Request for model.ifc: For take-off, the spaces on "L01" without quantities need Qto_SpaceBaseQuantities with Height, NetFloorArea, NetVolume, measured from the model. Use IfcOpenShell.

First a look at what the model holds.

```python
import ifcopenshell
import ifcopenshell.util.element
import ifcopenshell.util.unit

model = ifcopenshell.open("model.ifc")
print(model.schema)
for unit_type in ("LENGTHUNIT", "AREAUNIT", "VOLUMEUNIT"):
    print(unit_type, ifcopenshell.util.unit.calculate_unit_scale(model, unit_type))
storey = next(s for s in model.by_type("IfcBuildingStorey") if s.Name == "L01")
spaces = [e for e in ifcopenshell.util.element.get_decomposition(storey) if e.is_a("IfcSpace")]
for e in sorted(spaces, key=lambda e: e.id()):
    print(e.id(), e.is_a(), e.Name, list(ifcopenshell.util.element.get_psets(e, qtos_only=True)), sep=" | ")
```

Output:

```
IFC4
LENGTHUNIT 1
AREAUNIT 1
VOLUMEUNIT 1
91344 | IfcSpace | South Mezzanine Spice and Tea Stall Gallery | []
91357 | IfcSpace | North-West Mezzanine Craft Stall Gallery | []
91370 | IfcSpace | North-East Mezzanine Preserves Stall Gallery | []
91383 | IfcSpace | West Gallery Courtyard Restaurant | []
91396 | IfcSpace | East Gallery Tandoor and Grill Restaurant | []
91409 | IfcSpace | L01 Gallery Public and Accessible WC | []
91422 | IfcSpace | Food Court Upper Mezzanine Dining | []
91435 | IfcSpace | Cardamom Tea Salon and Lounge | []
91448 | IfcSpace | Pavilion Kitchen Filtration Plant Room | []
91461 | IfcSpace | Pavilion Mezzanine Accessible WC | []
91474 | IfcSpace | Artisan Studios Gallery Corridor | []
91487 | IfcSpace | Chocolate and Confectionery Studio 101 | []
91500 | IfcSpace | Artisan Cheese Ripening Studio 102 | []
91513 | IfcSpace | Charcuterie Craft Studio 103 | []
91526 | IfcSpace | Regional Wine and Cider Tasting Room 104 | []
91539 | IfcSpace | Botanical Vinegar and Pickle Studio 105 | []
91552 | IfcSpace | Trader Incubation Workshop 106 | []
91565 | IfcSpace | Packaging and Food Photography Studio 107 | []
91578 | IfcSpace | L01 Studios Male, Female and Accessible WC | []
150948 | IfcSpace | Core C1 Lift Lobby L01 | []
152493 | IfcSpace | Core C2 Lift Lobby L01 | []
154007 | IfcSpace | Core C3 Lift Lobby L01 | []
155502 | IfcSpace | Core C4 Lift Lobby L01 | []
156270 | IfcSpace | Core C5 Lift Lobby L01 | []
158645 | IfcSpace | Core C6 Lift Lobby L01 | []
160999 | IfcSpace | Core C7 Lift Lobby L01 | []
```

```python
import ifcopenshell
import ifcopenshell.api.pset
import ifcopenshell.geom
import ifcopenshell.util.element
import ifcopenshell.util.shape
import ifcopenshell.util.unit

model = ifcopenshell.open("model.ifc")
unit_scale = ifcopenshell.util.unit.calculate_unit_scale(model)
area_scale = ifcopenshell.util.unit.calculate_unit_scale(model, "AREAUNIT")
volume_scale = ifcopenshell.util.unit.calculate_unit_scale(model, "VOLUMEUNIT")
settings = ifcopenshell.geom.settings()

storey = next(s for s in model.by_type("IfcBuildingStorey") if s.Name == "L01")
spaces = [e for e in ifcopenshell.util.element.get_decomposition(storey) if e.is_a("IfcSpace")]

for e in sorted(spaces, key=lambda e: e.id()):
    if ifcopenshell.util.element.get_psets(e, qtos_only=True, should_inherit=False):
        continue
    # Geometry comes back in metres, in the element's own axes.
    shape = ifcopenshell.geom.create_shape(settings, e)
    values = {
        "Height": ifcopenshell.util.shape.get_z(shape.geometry) / unit_scale,
        "NetFloorArea": ifcopenshell.util.shape.get_footprint_area(shape.geometry) / area_scale,
        "NetVolume": ifcopenshell.util.shape.get_volume(shape.geometry) / volume_scale,
    }
    qto = ifcopenshell.api.pset.add_qto(model, product=e, name="Qto_SpaceBaseQuantities")
    ifcopenshell.api.pset.edit_qto(model, qto=qto, properties=values)
    print(e.id(), {k: round(v, 3) for k, v in values.items()})

model.write("model_updated.ifc")
```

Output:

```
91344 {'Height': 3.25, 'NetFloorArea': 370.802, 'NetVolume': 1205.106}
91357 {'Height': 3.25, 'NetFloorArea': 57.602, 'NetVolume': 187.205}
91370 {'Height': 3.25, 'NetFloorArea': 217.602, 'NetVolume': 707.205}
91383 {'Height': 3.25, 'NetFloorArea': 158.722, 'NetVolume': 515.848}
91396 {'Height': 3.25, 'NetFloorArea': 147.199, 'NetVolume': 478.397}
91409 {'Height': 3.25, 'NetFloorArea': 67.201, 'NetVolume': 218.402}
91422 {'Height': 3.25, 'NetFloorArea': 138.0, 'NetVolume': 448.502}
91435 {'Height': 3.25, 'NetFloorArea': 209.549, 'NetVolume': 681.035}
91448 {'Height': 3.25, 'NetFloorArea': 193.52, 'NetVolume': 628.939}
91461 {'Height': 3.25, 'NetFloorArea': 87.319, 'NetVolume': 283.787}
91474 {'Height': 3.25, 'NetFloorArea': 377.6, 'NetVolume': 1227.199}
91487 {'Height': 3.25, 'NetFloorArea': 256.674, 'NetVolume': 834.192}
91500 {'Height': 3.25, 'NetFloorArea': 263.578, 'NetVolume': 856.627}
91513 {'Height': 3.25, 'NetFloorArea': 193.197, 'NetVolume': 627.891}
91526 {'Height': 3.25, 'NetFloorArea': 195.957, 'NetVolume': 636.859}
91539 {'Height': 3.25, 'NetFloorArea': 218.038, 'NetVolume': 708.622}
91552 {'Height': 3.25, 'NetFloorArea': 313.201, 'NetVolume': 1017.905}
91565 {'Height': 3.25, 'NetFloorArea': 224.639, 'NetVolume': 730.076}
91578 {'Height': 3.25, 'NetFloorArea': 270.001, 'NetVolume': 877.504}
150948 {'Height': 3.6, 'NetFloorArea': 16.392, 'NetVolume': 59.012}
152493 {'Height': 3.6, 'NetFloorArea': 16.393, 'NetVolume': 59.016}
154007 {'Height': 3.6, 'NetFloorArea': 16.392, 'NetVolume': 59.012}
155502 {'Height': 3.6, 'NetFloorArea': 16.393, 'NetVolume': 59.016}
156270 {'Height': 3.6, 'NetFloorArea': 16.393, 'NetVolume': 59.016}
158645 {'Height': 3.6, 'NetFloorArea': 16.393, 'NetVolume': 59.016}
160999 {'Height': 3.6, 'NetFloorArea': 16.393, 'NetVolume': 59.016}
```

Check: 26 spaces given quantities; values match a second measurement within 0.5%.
